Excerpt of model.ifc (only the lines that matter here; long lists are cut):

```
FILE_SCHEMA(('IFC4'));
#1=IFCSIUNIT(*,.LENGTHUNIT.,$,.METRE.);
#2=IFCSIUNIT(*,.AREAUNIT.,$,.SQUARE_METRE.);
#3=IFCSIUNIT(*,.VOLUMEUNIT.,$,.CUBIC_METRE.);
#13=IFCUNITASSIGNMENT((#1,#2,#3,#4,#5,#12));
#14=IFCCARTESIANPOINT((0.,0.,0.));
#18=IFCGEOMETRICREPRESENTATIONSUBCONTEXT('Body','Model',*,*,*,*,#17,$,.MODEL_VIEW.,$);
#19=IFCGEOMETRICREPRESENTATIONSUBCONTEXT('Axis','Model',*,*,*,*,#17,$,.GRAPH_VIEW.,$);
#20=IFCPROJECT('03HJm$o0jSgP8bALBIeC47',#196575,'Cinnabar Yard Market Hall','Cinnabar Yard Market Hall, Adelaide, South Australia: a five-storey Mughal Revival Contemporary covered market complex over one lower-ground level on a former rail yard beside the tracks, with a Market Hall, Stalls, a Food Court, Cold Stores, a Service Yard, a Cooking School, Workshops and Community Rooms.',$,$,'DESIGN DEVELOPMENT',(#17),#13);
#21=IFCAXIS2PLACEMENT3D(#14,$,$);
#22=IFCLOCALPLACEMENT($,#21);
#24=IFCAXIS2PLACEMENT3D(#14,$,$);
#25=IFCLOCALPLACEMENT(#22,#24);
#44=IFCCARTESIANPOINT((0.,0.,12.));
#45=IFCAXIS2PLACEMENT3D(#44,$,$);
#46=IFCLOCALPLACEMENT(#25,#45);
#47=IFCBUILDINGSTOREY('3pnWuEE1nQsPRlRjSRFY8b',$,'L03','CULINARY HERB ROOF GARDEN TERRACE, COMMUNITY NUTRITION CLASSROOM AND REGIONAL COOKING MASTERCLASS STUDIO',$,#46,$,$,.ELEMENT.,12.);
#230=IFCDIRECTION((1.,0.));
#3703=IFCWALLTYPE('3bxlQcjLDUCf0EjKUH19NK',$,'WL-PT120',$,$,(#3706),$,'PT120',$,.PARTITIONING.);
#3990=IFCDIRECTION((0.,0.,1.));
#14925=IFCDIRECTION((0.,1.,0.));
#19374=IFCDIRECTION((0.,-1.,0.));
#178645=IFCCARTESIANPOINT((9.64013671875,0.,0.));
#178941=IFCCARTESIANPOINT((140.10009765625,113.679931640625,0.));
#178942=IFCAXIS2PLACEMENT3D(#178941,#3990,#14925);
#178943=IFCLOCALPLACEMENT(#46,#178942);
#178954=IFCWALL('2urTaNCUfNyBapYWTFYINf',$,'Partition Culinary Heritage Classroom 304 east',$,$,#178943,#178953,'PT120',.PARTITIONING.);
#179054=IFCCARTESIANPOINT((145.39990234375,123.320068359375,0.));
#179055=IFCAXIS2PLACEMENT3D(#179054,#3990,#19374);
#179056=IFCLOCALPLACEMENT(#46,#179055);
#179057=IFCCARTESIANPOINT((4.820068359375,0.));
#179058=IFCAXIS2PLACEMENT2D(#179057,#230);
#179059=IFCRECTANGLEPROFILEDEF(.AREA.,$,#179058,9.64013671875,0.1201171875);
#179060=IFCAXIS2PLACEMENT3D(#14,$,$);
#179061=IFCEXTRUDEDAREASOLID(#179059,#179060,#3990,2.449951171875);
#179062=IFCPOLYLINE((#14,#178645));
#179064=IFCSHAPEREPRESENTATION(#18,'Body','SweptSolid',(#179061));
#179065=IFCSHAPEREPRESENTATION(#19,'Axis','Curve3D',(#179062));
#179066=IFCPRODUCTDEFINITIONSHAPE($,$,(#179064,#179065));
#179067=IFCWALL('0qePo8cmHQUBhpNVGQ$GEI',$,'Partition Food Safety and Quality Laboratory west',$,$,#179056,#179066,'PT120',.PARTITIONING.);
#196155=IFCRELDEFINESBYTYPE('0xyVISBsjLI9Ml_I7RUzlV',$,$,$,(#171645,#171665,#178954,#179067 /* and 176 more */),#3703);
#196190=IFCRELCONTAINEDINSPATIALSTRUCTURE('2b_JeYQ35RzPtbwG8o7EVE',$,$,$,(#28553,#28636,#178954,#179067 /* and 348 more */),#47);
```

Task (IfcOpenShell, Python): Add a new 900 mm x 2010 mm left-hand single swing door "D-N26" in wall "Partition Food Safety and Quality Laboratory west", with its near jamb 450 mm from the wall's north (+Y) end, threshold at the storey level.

```python
import numpy as np
import ifcopenshell
import ifcopenshell.api.feature
import ifcopenshell.api.geometry
import ifcopenshell.api.root
import ifcopenshell.api.spatial
import ifcopenshell.geom
import ifcopenshell.util.element
import ifcopenshell.util.placement
import ifcopenshell.util.representation
import ifcopenshell.util.shape
import ifcopenshell.util.unit

model = ifcopenshell.open("model.ifc")
unit_scale = ifcopenshell.util.unit.calculate_unit_scale(model)
settings = ifcopenshell.geom.settings()


def volume(element):
    """Net volume in cubic metres, openings subtracted."""
    shape = ifcopenshell.geom.create_shape(settings, element)
    return ifcopenshell.util.shape.get_volume(shape.geometry)


wall = model.by_guid("0qePo8cmHQUBhpNVGQ$GEI")
storey = ifcopenshell.util.element.get_container(wall, ifc_class="IfcBuildingStorey")
context = ifcopenshell.util.representation.get_context(model, "Model", "Body", "MODEL_VIEW")
before = volume(wall)

width, height, from_end, sill = 0.9, 2.01, 0.45, 0.0  # metres

# The wall runs along its own X axis, and the end named is its -X end.
wall_shape = ifcopenshell.geom.create_shape(settings, wall)
x, y, z = ifcopenshell.util.shape.get_vertices(wall_shape.geometry).T
start = x.min() + from_end
face, thickness = float(y.min()), float(y.max() - y.min())
wall_matrix = ifcopenshell.util.placement.get_local_placement(wall.ObjectPlacement)
level = ifcopenshell.util.placement.get_local_placement(storey.ObjectPlacement)[2, 3]


def in_wall(x, y):
    """Placement at x, y metres in the wall's axes, at sill height."""
    matrix = wall_matrix.copy()
    matrix[:, 3] = wall_matrix @ np.array([x / unit_scale, y / unit_scale, 0.0, 1.0])
    matrix[2, 3] = level + sill / unit_scale
    return matrix


# Opening: a box that overshoots both wall faces by 50 mm.
opening = ifcopenshell.api.root.create_entity(model, ifc_class="IfcOpeningElement", predefined_type="OPENING")
box = ifcopenshell.api.geometry.add_wall_representation(
    model, context=context, length=width, height=height, thickness=thickness + 0.1
)
ifcopenshell.api.geometry.assign_representation(model, product=opening, representation=box)
ifcopenshell.api.geometry.edit_object_placement(model, product=opening, matrix=in_wall(start, face - 0.05), is_si=False)
ifcopenshell.api.feature.add_feature(model, feature=opening, element=wall)

door = ifcopenshell.api.root.create_entity(model, ifc_class="IfcDoor", name="D-N26", predefined_type="DOOR")
door.OverallWidth, door.OverallHeight = width / unit_scale, height / unit_scale
door.OperationType = "SINGLE_SWING_LEFT"
body = ifcopenshell.api.geometry.add_door_representation(
    model,
    context=context,
    overall_width=door.OverallWidth,
    overall_height=door.OverallHeight,
    operation_type="SINGLE_SWING_LEFT",
    lining_properties={"LiningDepth": thickness / unit_scale, "ThresholdDepth": thickness / unit_scale},
)
ifcopenshell.api.geometry.assign_representation(model, product=door, representation=body)
ifcopenshell.api.spatial.assign_container(model, products=[door], relating_structure=storey)
ifcopenshell.api.feature.add_filling(model, opening=opening, element=door)

# The lining spans the wall, so the door starts at the wall face.
ifcopenshell.api.geometry.edit_object_placement(model, product=door, matrix=in_wall(start, face), is_si=False)

after = volume(wall)

print(f"wall volume {before:.3f} -> {after:.3f} m3")

model.write("model_rev.ifc")
```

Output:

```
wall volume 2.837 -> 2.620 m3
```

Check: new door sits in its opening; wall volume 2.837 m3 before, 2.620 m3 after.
